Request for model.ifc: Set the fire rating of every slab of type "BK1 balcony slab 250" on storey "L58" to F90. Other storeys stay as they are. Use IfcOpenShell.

First a look at what the model holds.

```python
import ifcopenshell
import ifcopenshell.util.element

model = ifcopenshell.open("model.ifc")
print(model.schema)
storey = next(s for s in model.by_type("IfcBuildingStorey") if s.Name == "L58")
slabs = [e for e in ifcopenshell.util.element.get_decomposition(storey) if e.is_a("IfcSlab")]
seen = {}
for e in slabs:
    element_type = ifcopenshell.util.element.get_type(e)
    key = (element_type.Name if element_type != e and element_type else None, ifcopenshell.util.element.get_pset(e, "Pset_SlabCommon", "FireRating"))
    seen[key] = seen.get(key, 0) + 1
for (name, value), count in sorted(seen.items(), key=str):
    print(count, "x", name, "|", value)
```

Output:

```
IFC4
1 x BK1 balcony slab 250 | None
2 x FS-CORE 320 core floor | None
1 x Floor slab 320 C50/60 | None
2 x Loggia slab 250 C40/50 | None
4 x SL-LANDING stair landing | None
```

```python
import ifcopenshell
import ifcopenshell.api.pset
import ifcopenshell.util.element

model = ifcopenshell.open("model.ifc")

storey = next(s for s in model.by_type("IfcBuildingStorey") if s.Name == "L58")
slabs = [e for e in ifcopenshell.util.element.get_decomposition(storey) if e.is_a("IfcSlab")]

count = 0
for e in slabs:
    element_type = ifcopenshell.util.element.get_type(e)
    if element_type in (None, e) or element_type.Name != "BK1 balcony slab 250":
        continue
    found = ifcopenshell.util.element.get_pset(e, "Pset_SlabCommon", should_inherit=False)
    if found:
        pset = model.by_id(found["id"])
        if len(ifcopenshell.util.element.get_elements_by_pset(pset)) > 1:
            pset = ifcopenshell.api.pset.unshare_pset(model, products=[e], pset=pset)[0]
    else:
        pset = ifcopenshell.api.pset.add_pset(model, product=e, name="Pset_SlabCommon")
    ifcopenshell.api.pset.edit_pset(model, pset=pset, properties={"FireRating": "F90"})
    count += 1

print(count, "slabs updated")

model.write("model_v2.ifc")
```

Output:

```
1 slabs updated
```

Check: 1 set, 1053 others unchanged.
